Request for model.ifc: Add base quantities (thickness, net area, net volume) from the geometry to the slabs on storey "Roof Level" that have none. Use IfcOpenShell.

First a look at what the model holds.

```python
import ifcopenshell
import ifcopenshell.util.element
import ifcopenshell.util.unit

model = ifcopenshell.open("model.ifc")
print(model.schema)
for unit_type in ("LENGTHUNIT", "AREAUNIT", "VOLUMEUNIT"):
    print(unit_type, ifcopenshell.util.unit.calculate_unit_scale(model, unit_type))
storey = next(s for s in model.by_type("IfcBuildingStorey") if s.Name == "Roof Level")
slabs = [e for e in ifcopenshell.util.element.get_decomposition(storey) if e.is_a("IfcSlab")]
for e in sorted(slabs, key=lambda e: e.id()):
    print(e.id(), e.is_a(), e.Name, list(ifcopenshell.util.element.get_psets(e, qtos_only=True)), sep=" | ")
```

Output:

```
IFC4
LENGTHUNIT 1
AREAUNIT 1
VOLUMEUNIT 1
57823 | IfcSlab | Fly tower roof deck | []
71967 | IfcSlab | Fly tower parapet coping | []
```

```python
import ifcopenshell
import ifcopenshell.api.pset
import ifcopenshell.geom
import ifcopenshell.util.element
import ifcopenshell.util.shape
import ifcopenshell.util.unit

model = ifcopenshell.open("model.ifc")
unit_scale = ifcopenshell.util.unit.calculate_unit_scale(model)
area_scale = ifcopenshell.util.unit.calculate_unit_scale(model, "AREAUNIT")
volume_scale = ifcopenshell.util.unit.calculate_unit_scale(model, "VOLUMEUNIT")
settings = ifcopenshell.geom.settings()

storey = next(s for s in model.by_type("IfcBuildingStorey") if s.Name == "Roof Level")
slabs = [e for e in ifcopenshell.util.element.get_decomposition(storey) if e.is_a("IfcSlab")]

for e in sorted(slabs, key=lambda e: e.id()):
    if ifcopenshell.util.element.get_psets(e, qtos_only=True, should_inherit=False):
        continue
    # Geometry comes back in metres, in the element's own axes.
    shape = ifcopenshell.geom.create_shape(settings, e)
    values = {
        "Width": ifcopenshell.util.shape.get_z(shape.geometry) / unit_scale,
        "NetArea": ifcopenshell.util.shape.get_footprint_area(shape.geometry) / area_scale,
        "NetVolume": ifcopenshell.util.shape.get_volume(shape.geometry) / volume_scale,
    }
    qto = ifcopenshell.api.pset.add_qto(model, product=e, name="Qto_SlabBaseQuantities")
    ifcopenshell.api.pset.edit_qto(model, qto=qto, properties=values)
    print(e.id(), {k: round(v, 3) for k, v in values.items()})

model.write("model_v2.ifc")
```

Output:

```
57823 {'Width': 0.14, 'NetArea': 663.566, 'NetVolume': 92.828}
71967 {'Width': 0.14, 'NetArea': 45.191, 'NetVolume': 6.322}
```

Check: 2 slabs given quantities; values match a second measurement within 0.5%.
